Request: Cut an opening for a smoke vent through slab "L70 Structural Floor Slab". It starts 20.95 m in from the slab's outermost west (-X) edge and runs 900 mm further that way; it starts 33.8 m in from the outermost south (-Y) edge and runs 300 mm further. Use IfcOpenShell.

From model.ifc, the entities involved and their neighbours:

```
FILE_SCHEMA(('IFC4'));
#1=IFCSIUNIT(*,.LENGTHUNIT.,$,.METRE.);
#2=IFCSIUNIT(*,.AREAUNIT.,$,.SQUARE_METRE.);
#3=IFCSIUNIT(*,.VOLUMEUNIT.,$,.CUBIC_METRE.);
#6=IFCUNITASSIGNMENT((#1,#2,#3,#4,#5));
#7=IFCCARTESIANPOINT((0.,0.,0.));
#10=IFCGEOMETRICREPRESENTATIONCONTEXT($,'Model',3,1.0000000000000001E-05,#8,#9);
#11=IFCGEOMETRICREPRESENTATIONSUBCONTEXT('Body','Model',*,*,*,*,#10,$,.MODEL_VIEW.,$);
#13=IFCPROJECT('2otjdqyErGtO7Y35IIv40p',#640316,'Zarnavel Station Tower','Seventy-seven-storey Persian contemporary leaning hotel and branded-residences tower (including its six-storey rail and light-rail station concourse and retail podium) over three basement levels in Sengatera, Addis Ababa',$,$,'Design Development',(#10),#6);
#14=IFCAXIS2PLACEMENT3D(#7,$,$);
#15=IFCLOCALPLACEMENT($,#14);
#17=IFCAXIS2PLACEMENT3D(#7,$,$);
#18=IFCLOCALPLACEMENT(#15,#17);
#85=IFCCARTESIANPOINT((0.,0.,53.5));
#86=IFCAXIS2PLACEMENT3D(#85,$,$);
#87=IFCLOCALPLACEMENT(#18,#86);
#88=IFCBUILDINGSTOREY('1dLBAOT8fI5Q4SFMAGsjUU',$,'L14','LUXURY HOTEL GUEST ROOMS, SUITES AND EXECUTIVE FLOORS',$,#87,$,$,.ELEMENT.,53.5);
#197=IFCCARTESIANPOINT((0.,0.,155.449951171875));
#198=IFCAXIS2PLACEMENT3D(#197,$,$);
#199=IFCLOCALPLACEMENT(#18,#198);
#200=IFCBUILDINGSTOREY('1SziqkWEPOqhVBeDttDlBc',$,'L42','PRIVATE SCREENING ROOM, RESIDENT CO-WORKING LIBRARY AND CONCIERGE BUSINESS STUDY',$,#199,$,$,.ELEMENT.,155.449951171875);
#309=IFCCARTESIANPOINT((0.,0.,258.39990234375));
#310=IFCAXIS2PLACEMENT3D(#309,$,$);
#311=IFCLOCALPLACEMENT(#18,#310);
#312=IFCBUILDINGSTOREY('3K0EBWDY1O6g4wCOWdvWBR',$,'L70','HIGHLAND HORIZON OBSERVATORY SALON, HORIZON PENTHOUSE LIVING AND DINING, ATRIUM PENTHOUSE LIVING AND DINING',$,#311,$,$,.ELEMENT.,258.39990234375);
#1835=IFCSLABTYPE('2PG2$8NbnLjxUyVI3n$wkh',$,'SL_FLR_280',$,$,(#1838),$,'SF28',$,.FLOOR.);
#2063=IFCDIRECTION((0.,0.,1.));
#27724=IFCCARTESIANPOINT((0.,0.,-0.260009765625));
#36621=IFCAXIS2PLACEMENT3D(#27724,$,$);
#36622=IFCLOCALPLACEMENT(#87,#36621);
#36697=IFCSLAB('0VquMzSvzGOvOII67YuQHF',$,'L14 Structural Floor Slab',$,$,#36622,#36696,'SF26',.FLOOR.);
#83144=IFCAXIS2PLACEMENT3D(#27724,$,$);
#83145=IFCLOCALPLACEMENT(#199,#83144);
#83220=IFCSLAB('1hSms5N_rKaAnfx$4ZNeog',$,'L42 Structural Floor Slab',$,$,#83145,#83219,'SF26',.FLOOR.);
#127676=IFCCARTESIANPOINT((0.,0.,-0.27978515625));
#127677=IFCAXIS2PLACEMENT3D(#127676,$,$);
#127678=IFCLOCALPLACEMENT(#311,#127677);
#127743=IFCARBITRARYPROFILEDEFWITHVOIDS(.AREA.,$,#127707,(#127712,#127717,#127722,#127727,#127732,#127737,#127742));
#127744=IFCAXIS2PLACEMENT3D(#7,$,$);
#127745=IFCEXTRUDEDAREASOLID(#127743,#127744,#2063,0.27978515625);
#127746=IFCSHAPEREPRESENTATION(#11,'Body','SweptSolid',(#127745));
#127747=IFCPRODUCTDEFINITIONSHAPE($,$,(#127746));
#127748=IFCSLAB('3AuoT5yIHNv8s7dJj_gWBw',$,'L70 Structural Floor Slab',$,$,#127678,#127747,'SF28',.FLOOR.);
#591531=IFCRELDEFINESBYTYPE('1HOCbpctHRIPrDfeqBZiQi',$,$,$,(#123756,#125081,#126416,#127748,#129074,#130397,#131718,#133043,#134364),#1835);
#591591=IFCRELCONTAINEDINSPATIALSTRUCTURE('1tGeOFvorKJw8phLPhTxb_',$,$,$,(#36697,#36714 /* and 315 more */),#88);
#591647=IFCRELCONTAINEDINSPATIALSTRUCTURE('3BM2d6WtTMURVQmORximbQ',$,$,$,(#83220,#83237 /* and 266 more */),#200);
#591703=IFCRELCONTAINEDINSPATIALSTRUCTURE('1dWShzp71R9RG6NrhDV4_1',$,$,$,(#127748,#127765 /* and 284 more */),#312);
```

```python
import numpy as np
import ifcopenshell
import ifcopenshell.api.feature
import ifcopenshell.api.geometry
import ifcopenshell.api.root
import ifcopenshell.geom
import ifcopenshell.util.placement
import ifcopenshell.util.representation
import ifcopenshell.util.shape
import ifcopenshell.util.unit

model = ifcopenshell.open("model.ifc")
unit_scale = ifcopenshell.util.unit.calculate_unit_scale(model)
settings = ifcopenshell.geom.settings()


def volume(element):
    """Net volume in cubic metres, openings subtracted."""
    shape = ifcopenshell.geom.create_shape(settings, element)
    return ifcopenshell.util.shape.get_volume(shape.geometry)


slab = model.by_guid("3AuoT5yIHNv8s7dJj_gWBw")
before = volume(slab)

# Extent in the slab's own axes, in metres. The edges named are its -X and -Y sides.
slab_shape = ifcopenshell.geom.create_shape(settings, slab)
vertices = ifcopenshell.util.shape.get_vertices(slab_shape.geometry)
x_min, y_min, bottom = vertices.min(axis=0)
top = vertices[:, 2].max()

opening = ifcopenshell.api.root.create_entity(model, ifc_class="IfcOpeningElement", name="Smoke vent opening", predefined_type="OPENING")
context = ifcopenshell.util.representation.get_context(model, "Model", "Body", "MODEL_VIEW")
width, depth = 0.9, 0.3
outline = [(0.0, 0.0), (width, 0.0), (width, depth), (0.0, depth), (0.0, 0.0)]
# Overshoot both faces by 50 mm so the cut is clean.
shape = ifcopenshell.api.geometry.add_slab_representation(
    model, context=context, depth=top - bottom + 0.1, polyline=outline
)
ifcopenshell.api.geometry.assign_representation(model, product=opening, representation=shape)

matrix = ifcopenshell.util.placement.get_local_placement(slab.ObjectPlacement)
matrix[:, 3] = matrix @ np.append(np.array([x_min + 20.95, y_min + 33.8, bottom - 0.05]) / unit_scale, 1.0)
ifcopenshell.api.geometry.edit_object_placement(model, product=opening, matrix=matrix, is_si=False)
ifcopenshell.api.feature.add_feature(model, feature=opening, element=slab)

after = volume(slab)

print(f"slab volume {before:.3f} -> {after:.3f} m3")

model.write("model-out.ifc")
```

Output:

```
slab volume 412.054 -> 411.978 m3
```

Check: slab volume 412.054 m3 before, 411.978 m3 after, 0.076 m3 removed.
